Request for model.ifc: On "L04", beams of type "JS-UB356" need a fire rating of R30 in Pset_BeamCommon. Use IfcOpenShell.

First a look at what the model holds.

```python
import ifcopenshell
import ifcopenshell.util.element

model = ifcopenshell.open("model.ifc")
print(model.schema)
storey = next(s for s in model.by_type("IfcBuildingStorey") if s.Name == "L04")
beams = [e for e in ifcopenshell.util.element.get_decomposition(storey) if e.is_a("IfcBeam")]
seen = {}
for e in beams:
    element_type = ifcopenshell.util.element.get_type(e)
    key = (element_type.Name if element_type != e and element_type else None, ifcopenshell.util.element.get_pset(e, "Pset_BeamCommon", "FireRating"))
    seen[key] = seen.get(key, 0) + 1
for (name, value), count in sorted(seen.items(), key=str):
    print(count, "x", name, "|", value)
```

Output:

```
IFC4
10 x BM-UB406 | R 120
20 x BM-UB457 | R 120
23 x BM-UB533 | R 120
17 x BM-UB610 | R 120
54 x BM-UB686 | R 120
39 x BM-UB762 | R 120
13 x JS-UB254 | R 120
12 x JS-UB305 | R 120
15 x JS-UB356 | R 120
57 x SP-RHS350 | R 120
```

```python
import ifcopenshell
import ifcopenshell.api.pset
import ifcopenshell.util.element

model = ifcopenshell.open("model.ifc")

storey = next(s for s in model.by_type("IfcBuildingStorey") if s.Name == "L04")
beams = [e for e in ifcopenshell.util.element.get_decomposition(storey) if e.is_a("IfcBeam")]

count = 0
for e in beams:
    element_type = ifcopenshell.util.element.get_type(e)
    if element_type in (None, e) or element_type.Name != "JS-UB356":
        continue
    # add_pset returns the element's existing set when there is one.
    pset = ifcopenshell.api.pset.add_pset(model, product=e, name="Pset_BeamCommon")
    ifcopenshell.api.pset.edit_pset(model, pset=pset, properties={"FireRating": "R30"})
    count += 1

print(count, "beams updated")

model.write("model-out.ifc")
```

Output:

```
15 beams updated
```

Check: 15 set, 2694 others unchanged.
